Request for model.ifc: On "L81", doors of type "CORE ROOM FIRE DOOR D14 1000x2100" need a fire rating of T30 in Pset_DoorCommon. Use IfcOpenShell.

First a look at what the model holds.

```python
import ifcopenshell
import ifcopenshell.util.element

model = ifcopenshell.open("model.ifc")
print(model.schema)
storey = next(s for s in model.by_type("IfcBuildingStorey") if s.Name == "L81")
doors = [e for e in ifcopenshell.util.element.get_decomposition(storey) if e.is_a("IfcDoor")]
seen = {}
for e in doors:
    element_type = ifcopenshell.util.element.get_type(e)
    key = (element_type.Name if element_type != e and element_type else None, ifcopenshell.util.element.get_pset(e, "Pset_DoorCommon", "FireRating"))
    seen[key] = seen.get(key, 0) + 1
for (name, value), count in sorted(seen.items(), key=str):
    print(count, "x", name, "|", value)
```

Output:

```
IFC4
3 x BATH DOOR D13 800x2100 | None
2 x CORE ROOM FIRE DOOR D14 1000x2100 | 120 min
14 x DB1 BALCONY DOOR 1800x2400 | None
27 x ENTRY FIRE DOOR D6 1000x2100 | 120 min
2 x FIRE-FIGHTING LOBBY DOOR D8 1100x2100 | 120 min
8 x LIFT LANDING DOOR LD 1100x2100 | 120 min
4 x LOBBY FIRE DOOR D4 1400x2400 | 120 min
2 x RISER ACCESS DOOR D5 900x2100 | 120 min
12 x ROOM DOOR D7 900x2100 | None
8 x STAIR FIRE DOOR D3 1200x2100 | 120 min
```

```python
import ifcopenshell
import ifcopenshell.api.pset
import ifcopenshell.util.element

model = ifcopenshell.open("model.ifc")

storey = next(s for s in model.by_type("IfcBuildingStorey") if s.Name == "L81")
doors = [e for e in ifcopenshell.util.element.get_decomposition(storey) if e.is_a("IfcDoor")]

count = 0
for e in doors:
    element_type = ifcopenshell.util.element.get_type(e)
    if element_type in (None, e) or element_type.Name != "CORE ROOM FIRE DOOR D14 1000x2100":
        continue
    # add_pset returns the element's existing set when there is one.
    pset = ifcopenshell.api.pset.add_pset(model, product=e, name="Pset_DoorCommon")
    ifcopenshell.api.pset.edit_pset(model, pset=pset, properties={"FireRating": "T30"})
    count += 1

print(count, "doors updated")

model.write("model_edited.ifc")
```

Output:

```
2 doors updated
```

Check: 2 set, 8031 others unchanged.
